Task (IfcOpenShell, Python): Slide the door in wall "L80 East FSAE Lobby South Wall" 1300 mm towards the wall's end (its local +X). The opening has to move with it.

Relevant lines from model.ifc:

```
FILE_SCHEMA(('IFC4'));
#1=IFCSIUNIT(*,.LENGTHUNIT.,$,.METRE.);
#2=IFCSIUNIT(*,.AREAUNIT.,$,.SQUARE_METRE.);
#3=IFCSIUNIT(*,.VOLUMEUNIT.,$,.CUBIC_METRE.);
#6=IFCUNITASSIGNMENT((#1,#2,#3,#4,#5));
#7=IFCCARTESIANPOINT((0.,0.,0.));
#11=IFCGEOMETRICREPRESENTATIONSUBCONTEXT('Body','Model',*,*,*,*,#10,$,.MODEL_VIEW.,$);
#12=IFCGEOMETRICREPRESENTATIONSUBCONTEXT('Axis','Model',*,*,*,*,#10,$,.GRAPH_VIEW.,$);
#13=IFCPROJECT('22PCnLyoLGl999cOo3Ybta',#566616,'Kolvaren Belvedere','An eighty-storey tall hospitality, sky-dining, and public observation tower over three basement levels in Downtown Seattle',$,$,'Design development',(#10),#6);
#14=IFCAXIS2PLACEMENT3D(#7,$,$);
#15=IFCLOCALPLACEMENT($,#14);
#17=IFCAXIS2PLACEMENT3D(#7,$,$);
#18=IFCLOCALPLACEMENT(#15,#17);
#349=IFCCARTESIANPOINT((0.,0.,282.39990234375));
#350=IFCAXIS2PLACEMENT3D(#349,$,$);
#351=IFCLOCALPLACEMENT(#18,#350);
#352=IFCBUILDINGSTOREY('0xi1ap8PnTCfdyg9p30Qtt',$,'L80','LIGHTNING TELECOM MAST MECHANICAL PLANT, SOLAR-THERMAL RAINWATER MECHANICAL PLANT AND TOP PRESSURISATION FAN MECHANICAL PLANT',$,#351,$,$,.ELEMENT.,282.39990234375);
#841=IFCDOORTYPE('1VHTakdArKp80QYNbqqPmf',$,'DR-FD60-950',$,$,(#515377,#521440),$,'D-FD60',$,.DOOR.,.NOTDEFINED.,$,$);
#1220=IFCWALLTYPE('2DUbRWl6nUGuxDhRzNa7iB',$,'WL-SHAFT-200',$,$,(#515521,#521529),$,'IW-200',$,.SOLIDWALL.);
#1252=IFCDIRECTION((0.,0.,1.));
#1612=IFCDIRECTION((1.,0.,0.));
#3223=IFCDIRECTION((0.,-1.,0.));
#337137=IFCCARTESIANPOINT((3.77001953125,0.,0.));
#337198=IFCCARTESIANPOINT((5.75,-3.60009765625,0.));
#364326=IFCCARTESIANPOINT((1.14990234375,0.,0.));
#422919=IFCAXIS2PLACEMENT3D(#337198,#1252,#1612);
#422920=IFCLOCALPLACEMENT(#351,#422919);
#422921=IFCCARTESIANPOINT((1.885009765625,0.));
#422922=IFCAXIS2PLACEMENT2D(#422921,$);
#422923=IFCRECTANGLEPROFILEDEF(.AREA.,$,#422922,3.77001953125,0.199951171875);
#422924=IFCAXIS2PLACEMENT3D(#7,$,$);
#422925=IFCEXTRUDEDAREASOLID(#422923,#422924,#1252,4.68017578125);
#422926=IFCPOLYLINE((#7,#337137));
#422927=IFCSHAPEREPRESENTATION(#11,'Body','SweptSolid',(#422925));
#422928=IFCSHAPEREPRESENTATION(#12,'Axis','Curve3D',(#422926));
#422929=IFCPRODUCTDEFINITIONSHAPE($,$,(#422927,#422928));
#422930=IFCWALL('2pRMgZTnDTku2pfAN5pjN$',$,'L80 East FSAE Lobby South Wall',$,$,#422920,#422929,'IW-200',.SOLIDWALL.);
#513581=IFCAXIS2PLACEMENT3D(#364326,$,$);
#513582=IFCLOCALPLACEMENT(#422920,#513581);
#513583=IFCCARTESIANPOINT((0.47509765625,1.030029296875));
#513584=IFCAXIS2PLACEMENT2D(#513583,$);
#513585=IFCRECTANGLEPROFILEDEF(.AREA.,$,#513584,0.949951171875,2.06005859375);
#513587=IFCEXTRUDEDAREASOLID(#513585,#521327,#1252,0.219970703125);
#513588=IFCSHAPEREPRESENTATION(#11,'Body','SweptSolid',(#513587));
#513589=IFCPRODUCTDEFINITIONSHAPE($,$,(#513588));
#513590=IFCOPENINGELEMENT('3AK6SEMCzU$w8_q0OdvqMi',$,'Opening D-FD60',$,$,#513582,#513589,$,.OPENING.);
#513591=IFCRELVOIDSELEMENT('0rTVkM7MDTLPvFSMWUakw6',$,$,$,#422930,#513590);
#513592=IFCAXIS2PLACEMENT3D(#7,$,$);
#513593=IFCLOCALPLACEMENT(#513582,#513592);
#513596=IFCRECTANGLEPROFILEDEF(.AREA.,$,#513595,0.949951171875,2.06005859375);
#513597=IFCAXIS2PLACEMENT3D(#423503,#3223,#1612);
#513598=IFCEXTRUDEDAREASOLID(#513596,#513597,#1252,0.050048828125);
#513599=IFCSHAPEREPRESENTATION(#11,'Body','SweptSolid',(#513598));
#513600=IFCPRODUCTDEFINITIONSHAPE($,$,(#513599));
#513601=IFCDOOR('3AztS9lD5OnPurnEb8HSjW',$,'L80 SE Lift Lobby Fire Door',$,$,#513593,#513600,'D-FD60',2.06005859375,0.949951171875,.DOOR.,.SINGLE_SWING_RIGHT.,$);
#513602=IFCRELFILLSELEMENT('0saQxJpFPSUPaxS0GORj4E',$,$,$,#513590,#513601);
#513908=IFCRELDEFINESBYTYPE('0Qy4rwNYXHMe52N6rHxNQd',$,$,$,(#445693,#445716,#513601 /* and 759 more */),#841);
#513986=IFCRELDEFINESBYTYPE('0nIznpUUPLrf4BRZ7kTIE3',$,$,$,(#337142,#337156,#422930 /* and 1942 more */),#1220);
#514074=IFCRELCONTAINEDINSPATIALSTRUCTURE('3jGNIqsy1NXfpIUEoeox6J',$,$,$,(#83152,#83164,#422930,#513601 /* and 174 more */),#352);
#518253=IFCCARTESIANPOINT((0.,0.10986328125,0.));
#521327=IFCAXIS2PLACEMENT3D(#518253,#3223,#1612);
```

```python
import ifcopenshell
import ifcopenshell.api.geometry
import ifcopenshell.util.placement
import ifcopenshell.util.unit

model = ifcopenshell.open("model.ifc")
unit_scale = ifcopenshell.util.unit.calculate_unit_scale(model)

door = model.by_guid("3AztS9lD5OnPurnEb8HSjW")
opening = door.FillsVoids[0].RelatingOpeningElement
wall = opening.VoidsElements[0].RelatingBuildingElement

wall_matrix = ifcopenshell.util.placement.get_local_placement(wall.ObjectPlacement)
shift = wall_matrix[:3, 0] * 1.3 / unit_scale
before = ifcopenshell.util.placement.get_local_placement(door.ObjectPlacement)[:3, 3].copy()

# The door is placed relative to its opening, so it follows when the opening moves.
matrix = ifcopenshell.util.placement.get_local_placement(opening.ObjectPlacement)
matrix[:3, 3] += shift
ifcopenshell.api.geometry.edit_object_placement(
    model, product=opening, matrix=matrix, is_si=False, should_transform_children=True
)

after = ifcopenshell.util.placement.get_local_placement(door.ObjectPlacement)[:3, 3]
print("door moved by", (after - before).round(3) + 0.0)

model.write("model_rev.ifc")
```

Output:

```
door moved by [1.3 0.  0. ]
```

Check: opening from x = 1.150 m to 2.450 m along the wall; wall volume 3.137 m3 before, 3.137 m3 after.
